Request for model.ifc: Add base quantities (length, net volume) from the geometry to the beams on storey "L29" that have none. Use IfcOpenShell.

First a look at what the model holds.

```python
import ifcopenshell
import ifcopenshell.util.element
import ifcopenshell.util.unit

model = ifcopenshell.open("model.ifc")
print(model.schema)
for unit_type in ("LENGTHUNIT", "AREAUNIT", "VOLUMEUNIT"):
    print(unit_type, ifcopenshell.util.unit.calculate_unit_scale(model, unit_type))
storey = next(s for s in model.by_type("IfcBuildingStorey") if s.Name == "L29")
beams = [e for e in ifcopenshell.util.element.get_decomposition(storey) if e.is_a("IfcBeam")]
for e in sorted(beams, key=lambda e: e.id()):
    print(e.id(), e.is_a(), e.Name, list(ifcopenshell.util.element.get_psets(e, qtos_only=True)), sep=" | ")
```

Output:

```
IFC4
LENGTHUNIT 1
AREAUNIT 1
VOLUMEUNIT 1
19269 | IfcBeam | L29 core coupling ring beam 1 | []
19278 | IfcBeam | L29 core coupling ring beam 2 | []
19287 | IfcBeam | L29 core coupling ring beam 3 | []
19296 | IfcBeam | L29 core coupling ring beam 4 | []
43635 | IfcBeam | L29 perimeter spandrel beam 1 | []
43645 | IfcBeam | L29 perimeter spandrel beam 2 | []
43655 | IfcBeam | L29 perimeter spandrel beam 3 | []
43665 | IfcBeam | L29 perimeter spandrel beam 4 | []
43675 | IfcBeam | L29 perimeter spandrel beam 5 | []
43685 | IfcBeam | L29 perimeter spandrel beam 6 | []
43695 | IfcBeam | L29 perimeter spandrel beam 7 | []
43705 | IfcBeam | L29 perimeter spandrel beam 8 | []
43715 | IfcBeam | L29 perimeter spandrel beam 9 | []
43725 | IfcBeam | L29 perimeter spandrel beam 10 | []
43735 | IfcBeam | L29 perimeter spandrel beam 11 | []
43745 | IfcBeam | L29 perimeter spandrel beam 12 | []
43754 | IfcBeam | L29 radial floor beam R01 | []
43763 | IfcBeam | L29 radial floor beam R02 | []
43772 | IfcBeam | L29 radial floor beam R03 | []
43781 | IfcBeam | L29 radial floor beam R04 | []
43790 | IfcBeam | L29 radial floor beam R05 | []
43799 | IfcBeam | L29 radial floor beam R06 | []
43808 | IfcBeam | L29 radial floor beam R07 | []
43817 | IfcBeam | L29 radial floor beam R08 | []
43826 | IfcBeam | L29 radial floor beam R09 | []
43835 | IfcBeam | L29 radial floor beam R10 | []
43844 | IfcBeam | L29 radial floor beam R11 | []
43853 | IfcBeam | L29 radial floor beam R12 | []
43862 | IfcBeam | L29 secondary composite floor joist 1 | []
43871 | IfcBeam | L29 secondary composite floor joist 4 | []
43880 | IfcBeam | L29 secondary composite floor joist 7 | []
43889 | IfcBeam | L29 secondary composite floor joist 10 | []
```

```python
import ifcopenshell
import ifcopenshell.api.pset
import ifcopenshell.geom
import ifcopenshell.util.element
import ifcopenshell.util.shape
import ifcopenshell.util.unit

model = ifcopenshell.open("model.ifc")
unit_scale = ifcopenshell.util.unit.calculate_unit_scale(model)
volume_scale = ifcopenshell.util.unit.calculate_unit_scale(model, "VOLUMEUNIT")
settings = ifcopenshell.geom.settings()

storey = next(s for s in model.by_type("IfcBuildingStorey") if s.Name == "L29")
beams = [e for e in ifcopenshell.util.element.get_decomposition(storey) if e.is_a("IfcBeam")]

for e in sorted(beams, key=lambda e: e.id()):
    if ifcopenshell.util.element.get_psets(e, qtos_only=True, should_inherit=False):
        continue
    # Geometry comes back in metres, in the element's own axes.
    shape = ifcopenshell.geom.create_shape(settings, e)
    values = {
        "Length": ifcopenshell.util.shape.get_max_xyz(shape.geometry) / unit_scale,
        "NetVolume": ifcopenshell.util.shape.get_volume(shape.geometry) / volume_scale,
    }
    qto = ifcopenshell.api.pset.add_qto(model, product=e, name="Qto_BeamBaseQuantities")
    ifcopenshell.api.pset.edit_qto(model, qto=qto, properties=values)
    print(e.id(), {k: round(v, 3) for k, v in values.items()})

model.write("model_edited.ifc")
```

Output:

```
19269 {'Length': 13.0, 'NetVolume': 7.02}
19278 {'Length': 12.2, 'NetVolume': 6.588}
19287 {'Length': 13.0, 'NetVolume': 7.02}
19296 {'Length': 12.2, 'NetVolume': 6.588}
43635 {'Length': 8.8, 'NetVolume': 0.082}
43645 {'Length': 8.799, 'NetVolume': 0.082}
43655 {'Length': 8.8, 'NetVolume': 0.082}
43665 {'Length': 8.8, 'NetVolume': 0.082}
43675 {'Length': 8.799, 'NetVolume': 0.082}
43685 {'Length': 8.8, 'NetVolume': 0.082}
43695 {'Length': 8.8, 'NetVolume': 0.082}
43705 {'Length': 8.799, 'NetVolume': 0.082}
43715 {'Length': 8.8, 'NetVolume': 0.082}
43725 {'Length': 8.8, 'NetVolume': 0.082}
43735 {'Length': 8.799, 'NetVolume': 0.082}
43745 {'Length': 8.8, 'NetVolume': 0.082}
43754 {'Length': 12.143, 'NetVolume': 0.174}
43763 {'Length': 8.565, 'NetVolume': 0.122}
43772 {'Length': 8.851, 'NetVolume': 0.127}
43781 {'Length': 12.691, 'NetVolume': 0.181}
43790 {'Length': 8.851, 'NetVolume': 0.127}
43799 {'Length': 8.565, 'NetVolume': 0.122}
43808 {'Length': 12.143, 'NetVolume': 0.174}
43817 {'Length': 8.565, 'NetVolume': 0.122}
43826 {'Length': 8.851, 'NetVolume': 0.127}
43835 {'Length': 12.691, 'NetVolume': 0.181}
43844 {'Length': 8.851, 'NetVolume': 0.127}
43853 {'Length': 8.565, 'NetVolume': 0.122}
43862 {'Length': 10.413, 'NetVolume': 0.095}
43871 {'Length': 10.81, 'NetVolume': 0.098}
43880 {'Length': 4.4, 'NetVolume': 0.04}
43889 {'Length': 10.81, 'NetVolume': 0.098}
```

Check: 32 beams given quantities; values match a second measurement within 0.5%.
